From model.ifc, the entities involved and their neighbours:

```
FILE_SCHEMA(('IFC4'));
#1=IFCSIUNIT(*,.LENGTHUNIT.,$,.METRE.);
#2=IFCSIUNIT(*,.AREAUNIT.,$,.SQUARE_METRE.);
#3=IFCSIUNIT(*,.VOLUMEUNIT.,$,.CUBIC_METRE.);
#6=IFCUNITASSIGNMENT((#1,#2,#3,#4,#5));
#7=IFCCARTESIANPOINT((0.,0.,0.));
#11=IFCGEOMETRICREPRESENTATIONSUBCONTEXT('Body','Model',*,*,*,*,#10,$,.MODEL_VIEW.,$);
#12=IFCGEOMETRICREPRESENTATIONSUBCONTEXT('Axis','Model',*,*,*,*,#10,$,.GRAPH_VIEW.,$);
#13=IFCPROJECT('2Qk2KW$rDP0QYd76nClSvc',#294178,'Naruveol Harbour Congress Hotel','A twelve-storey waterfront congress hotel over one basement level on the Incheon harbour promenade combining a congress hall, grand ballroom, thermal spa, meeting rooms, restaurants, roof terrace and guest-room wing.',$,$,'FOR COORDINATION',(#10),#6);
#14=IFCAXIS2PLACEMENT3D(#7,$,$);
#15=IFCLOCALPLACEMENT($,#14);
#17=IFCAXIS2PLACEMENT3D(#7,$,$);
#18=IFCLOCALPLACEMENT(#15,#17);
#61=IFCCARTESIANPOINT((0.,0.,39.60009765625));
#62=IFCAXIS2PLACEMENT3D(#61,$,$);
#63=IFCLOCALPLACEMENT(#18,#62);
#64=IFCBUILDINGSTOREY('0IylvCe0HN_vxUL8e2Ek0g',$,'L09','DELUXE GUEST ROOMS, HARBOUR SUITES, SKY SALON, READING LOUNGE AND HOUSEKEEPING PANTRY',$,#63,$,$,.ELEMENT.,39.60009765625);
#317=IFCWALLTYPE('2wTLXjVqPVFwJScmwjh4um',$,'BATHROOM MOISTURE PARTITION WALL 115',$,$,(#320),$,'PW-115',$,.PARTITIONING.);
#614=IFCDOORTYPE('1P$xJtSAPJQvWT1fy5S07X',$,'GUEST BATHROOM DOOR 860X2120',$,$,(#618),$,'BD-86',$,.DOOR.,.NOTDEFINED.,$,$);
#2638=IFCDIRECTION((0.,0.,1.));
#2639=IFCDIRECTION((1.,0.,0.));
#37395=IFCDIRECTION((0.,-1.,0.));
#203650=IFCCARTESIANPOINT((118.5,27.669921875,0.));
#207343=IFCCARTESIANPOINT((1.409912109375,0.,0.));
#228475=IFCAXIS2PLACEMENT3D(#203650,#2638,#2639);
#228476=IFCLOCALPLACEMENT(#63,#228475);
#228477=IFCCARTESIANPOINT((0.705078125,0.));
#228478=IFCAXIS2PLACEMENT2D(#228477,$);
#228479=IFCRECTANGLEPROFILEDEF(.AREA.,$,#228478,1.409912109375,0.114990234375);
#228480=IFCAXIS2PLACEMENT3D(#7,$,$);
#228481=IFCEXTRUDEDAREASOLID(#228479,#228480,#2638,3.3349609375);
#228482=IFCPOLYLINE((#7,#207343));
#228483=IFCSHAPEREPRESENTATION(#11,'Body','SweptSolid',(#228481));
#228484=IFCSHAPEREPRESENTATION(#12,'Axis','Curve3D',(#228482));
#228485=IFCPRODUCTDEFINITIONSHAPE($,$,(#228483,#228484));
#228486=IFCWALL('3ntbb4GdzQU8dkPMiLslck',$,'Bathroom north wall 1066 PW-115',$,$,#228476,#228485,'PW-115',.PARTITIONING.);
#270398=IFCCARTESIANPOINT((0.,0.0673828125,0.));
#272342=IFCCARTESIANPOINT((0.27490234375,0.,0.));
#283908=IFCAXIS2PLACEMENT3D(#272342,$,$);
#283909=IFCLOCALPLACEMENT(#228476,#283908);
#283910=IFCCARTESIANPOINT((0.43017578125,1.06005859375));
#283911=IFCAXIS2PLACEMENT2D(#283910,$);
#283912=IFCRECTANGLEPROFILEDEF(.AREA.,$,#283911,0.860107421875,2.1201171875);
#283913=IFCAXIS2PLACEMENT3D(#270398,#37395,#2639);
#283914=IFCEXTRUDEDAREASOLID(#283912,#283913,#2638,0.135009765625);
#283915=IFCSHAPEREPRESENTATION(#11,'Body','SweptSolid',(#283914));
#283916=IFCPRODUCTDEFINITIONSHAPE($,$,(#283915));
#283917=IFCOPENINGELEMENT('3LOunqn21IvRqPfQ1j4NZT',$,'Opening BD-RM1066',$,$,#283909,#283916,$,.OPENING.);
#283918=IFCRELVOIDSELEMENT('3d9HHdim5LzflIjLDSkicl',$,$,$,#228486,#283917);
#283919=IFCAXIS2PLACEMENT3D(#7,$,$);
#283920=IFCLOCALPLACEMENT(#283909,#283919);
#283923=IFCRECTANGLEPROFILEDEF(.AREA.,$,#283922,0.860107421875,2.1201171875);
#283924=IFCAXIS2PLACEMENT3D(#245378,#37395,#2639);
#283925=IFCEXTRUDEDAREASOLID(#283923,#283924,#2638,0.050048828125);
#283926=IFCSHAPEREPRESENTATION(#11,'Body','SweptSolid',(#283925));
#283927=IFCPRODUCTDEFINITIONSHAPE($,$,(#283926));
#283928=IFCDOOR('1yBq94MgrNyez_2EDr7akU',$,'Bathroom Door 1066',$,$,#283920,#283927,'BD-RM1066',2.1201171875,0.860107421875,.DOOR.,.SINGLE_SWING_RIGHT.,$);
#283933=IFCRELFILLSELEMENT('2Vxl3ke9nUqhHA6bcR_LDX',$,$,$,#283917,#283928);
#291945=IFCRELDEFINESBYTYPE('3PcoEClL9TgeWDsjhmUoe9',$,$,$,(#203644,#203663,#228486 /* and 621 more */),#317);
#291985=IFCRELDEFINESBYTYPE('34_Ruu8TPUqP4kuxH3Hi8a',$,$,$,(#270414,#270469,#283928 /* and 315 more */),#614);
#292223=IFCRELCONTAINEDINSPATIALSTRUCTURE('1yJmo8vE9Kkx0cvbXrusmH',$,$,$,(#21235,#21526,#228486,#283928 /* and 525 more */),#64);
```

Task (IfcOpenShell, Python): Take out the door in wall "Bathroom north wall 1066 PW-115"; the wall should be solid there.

```python
import ifcopenshell
import ifcopenshell.api.feature
import ifcopenshell.api.root
import ifcopenshell.geom
import ifcopenshell.util.shape

model = ifcopenshell.open("model.ifc")
settings = ifcopenshell.geom.settings()


def volume(element):
    """Net volume in cubic metres, openings subtracted."""
    shape = ifcopenshell.geom.create_shape(settings, element)
    return ifcopenshell.util.shape.get_volume(shape.geometry)


door = model.by_id(283928)
opening = door.FillsVoids[0].RelatingOpeningElement
wall = opening.VoidsElements[0].RelatingBuildingElement
before = volume(wall)

ifcopenshell.api.root.remove_product(model, product=door)
ifcopenshell.api.feature.remove_feature(model, feature=opening)

after = volume(wall)

print(f"wall volume {before:.3f} -> {after:.3f} m3")

model.write("model-out.ifc")
```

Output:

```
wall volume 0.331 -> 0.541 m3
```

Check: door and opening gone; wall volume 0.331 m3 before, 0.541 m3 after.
